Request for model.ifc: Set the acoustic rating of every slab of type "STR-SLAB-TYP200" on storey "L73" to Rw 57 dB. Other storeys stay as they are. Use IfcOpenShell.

First a look at what the model holds.

```python
import ifcopenshell
import ifcopenshell.util.element

model = ifcopenshell.open("model.ifc")
print(model.schema)
storey = next(s for s in model.by_type("IfcBuildingStorey") if s.Name == "L73")
slabs = [e for e in ifcopenshell.util.element.get_decomposition(storey) if e.is_a("IfcSlab")]
seen = {}
for e in slabs:
    element_type = ifcopenshell.util.element.get_type(e)
    key = (element_type.Name if element_type != e and element_type else None, ifcopenshell.util.element.get_pset(e, "Pset_SlabCommon", "AcousticRating"))
    seen[key] = seen.get(key, 0) + 1
for (name, value), count in sorted(seen.items(), key=str):
    print(count, "x", name, "|", value)
```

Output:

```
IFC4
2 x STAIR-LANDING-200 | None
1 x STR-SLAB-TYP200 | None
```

```python
import ifcopenshell
import ifcopenshell.api.pset
import ifcopenshell.util.element

model = ifcopenshell.open("model.ifc")

storey = next(s for s in model.by_type("IfcBuildingStorey") if s.Name == "L73")
slabs = [e for e in ifcopenshell.util.element.get_decomposition(storey) if e.is_a("IfcSlab")]

count = 0
for e in slabs:
    element_type = ifcopenshell.util.element.get_type(e)
    if element_type in (None, e) or element_type.Name != "STR-SLAB-TYP200":
        continue
    found = ifcopenshell.util.element.get_pset(e, "Pset_SlabCommon", should_inherit=False)
    if found:
        pset = model.by_id(found["id"])
        if len(ifcopenshell.util.element.get_elements_by_pset(pset)) > 1:
            pset = ifcopenshell.api.pset.unshare_pset(model, products=[e], pset=pset)[0]
    else:
        pset = ifcopenshell.api.pset.add_pset(model, product=e, name="Pset_SlabCommon")
    ifcopenshell.api.pset.edit_pset(model, pset=pset, properties={"AcousticRating": "Rw 57 dB"})
    count += 1

print(count, "slabs updated")

model.write("model-out.ifc")
```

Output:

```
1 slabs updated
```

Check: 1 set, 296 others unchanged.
